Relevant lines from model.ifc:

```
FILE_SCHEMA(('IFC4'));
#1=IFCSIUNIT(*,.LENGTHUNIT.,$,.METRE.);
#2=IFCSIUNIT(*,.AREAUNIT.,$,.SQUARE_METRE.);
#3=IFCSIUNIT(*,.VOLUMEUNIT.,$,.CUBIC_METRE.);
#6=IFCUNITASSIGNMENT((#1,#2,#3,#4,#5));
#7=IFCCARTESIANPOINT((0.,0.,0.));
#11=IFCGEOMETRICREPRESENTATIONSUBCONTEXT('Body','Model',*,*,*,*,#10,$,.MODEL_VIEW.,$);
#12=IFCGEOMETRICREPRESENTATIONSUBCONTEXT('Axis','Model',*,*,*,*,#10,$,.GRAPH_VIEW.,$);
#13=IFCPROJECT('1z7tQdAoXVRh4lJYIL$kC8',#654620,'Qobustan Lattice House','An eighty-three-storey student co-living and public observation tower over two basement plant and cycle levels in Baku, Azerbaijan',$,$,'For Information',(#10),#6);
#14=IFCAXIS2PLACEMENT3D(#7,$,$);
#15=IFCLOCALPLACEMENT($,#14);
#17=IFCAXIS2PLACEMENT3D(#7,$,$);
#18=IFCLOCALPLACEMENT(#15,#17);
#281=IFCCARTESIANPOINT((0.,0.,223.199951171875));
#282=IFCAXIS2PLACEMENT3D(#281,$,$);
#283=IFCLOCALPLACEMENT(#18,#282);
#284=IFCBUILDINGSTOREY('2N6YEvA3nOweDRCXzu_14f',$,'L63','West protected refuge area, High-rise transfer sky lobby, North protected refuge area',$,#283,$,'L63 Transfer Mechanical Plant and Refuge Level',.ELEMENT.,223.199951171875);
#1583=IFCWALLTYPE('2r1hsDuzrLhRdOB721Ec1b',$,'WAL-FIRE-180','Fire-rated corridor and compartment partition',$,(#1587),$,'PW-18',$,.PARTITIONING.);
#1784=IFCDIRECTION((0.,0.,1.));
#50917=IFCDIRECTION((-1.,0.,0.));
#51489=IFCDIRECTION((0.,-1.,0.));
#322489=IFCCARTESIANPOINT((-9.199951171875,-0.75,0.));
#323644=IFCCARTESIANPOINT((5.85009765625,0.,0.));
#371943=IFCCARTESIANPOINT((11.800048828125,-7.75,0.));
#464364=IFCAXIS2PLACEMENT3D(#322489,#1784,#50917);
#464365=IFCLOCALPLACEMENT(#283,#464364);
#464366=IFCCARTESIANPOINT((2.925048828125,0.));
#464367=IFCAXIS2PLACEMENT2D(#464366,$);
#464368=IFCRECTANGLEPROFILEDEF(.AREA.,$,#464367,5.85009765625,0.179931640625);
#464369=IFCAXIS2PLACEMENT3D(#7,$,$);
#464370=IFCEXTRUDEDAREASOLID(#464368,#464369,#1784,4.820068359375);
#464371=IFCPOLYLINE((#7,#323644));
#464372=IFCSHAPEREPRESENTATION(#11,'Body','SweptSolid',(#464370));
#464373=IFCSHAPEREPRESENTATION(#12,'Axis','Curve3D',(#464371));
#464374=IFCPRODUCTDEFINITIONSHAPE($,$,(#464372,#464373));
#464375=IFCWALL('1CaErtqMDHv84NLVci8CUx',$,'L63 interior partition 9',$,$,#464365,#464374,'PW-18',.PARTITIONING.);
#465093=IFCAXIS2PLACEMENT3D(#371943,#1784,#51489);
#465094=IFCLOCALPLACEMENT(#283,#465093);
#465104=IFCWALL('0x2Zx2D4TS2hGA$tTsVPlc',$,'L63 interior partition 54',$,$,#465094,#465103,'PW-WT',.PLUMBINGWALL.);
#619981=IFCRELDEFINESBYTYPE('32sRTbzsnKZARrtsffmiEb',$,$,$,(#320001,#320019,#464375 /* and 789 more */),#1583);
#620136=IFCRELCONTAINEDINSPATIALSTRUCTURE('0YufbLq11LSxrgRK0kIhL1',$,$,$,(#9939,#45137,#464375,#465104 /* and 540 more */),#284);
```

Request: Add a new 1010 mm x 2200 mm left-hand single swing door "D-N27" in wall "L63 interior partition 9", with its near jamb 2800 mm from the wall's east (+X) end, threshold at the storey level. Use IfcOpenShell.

```python
import numpy as np
import ifcopenshell
import ifcopenshell.api.feature
import ifcopenshell.api.geometry
import ifcopenshell.api.root
import ifcopenshell.api.spatial
import ifcopenshell.geom
import ifcopenshell.util.element
import ifcopenshell.util.placement
import ifcopenshell.util.representation
import ifcopenshell.util.shape
import ifcopenshell.util.unit

model = ifcopenshell.open("model.ifc")
unit_scale = ifcopenshell.util.unit.calculate_unit_scale(model)
settings = ifcopenshell.geom.settings()


def volume(element):
    """Net volume in cubic metres, openings subtracted."""
    shape = ifcopenshell.geom.create_shape(settings, element)
    return ifcopenshell.util.shape.get_volume(shape.geometry)


wall = model.by_guid("1CaErtqMDHv84NLVci8CUx")
storey = ifcopenshell.util.element.get_container(wall, ifc_class="IfcBuildingStorey")
context = ifcopenshell.util.representation.get_context(model, "Model", "Body", "MODEL_VIEW")
before = volume(wall)

width, height, from_end, sill = 1.01, 2.2, 2.8, 0.0  # metres

# The wall runs along its own X axis, and the end named is its -X end.
wall_shape = ifcopenshell.geom.create_shape(settings, wall)
x, y, z = ifcopenshell.util.shape.get_vertices(wall_shape.geometry).T
start = x.min() + from_end
face, thickness = float(y.min()), float(y.max() - y.min())
wall_matrix = ifcopenshell.util.placement.get_local_placement(wall.ObjectPlacement)
level = ifcopenshell.util.placement.get_local_placement(storey.ObjectPlacement)[2, 3]


def in_wall(x, y):
    """Placement at x, y metres in the wall's axes, at sill height."""
    matrix = wall_matrix.copy()
    matrix[:, 3] = wall_matrix @ np.array([x / unit_scale, y / unit_scale, 0.0, 1.0])
    matrix[2, 3] = level + sill / unit_scale
    return matrix


# Opening: a box that overshoots both wall faces by 50 mm.
opening = ifcopenshell.api.root.create_entity(model, ifc_class="IfcOpeningElement", predefined_type="OPENING")
box = ifcopenshell.api.geometry.add_wall_representation(
    model, context=context, length=width, height=height, thickness=thickness + 0.1
)
ifcopenshell.api.geometry.assign_representation(model, product=opening, representation=box)
ifcopenshell.api.geometry.edit_object_placement(model, product=opening, matrix=in_wall(start, face - 0.05), is_si=False)
ifcopenshell.api.feature.add_feature(model, feature=opening, element=wall)

door = ifcopenshell.api.root.create_entity(model, ifc_class="IfcDoor", name="D-N27", predefined_type="DOOR")
door.OverallWidth, door.OverallHeight = width / unit_scale, height / unit_scale
door.OperationType = "SINGLE_SWING_LEFT"
body = ifcopenshell.api.geometry.add_door_representation(
    model,
    context=context,
    overall_width=door.OverallWidth,
    overall_height=door.OverallHeight,
    operation_type="SINGLE_SWING_LEFT",
    lining_properties={"LiningDepth": thickness / unit_scale, "ThresholdDepth": thickness / unit_scale},
)
ifcopenshell.api.geometry.assign_representation(model, product=door, representation=body)
ifcopenshell.api.spatial.assign_container(model, products=[door], relating_structure=storey)
ifcopenshell.api.feature.add_filling(model, opening=opening, element=door)

# The lining spans the wall, so the door starts at the wall face.
ifcopenshell.api.geometry.edit_object_placement(model, product=door, matrix=in_wall(start, face), is_si=False)

after = volume(wall)

print(f"wall volume {before:.3f} -> {after:.3f} m3")

model.write("model_v2.ifc")
```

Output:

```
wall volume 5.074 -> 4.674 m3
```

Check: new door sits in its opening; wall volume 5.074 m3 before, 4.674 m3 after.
